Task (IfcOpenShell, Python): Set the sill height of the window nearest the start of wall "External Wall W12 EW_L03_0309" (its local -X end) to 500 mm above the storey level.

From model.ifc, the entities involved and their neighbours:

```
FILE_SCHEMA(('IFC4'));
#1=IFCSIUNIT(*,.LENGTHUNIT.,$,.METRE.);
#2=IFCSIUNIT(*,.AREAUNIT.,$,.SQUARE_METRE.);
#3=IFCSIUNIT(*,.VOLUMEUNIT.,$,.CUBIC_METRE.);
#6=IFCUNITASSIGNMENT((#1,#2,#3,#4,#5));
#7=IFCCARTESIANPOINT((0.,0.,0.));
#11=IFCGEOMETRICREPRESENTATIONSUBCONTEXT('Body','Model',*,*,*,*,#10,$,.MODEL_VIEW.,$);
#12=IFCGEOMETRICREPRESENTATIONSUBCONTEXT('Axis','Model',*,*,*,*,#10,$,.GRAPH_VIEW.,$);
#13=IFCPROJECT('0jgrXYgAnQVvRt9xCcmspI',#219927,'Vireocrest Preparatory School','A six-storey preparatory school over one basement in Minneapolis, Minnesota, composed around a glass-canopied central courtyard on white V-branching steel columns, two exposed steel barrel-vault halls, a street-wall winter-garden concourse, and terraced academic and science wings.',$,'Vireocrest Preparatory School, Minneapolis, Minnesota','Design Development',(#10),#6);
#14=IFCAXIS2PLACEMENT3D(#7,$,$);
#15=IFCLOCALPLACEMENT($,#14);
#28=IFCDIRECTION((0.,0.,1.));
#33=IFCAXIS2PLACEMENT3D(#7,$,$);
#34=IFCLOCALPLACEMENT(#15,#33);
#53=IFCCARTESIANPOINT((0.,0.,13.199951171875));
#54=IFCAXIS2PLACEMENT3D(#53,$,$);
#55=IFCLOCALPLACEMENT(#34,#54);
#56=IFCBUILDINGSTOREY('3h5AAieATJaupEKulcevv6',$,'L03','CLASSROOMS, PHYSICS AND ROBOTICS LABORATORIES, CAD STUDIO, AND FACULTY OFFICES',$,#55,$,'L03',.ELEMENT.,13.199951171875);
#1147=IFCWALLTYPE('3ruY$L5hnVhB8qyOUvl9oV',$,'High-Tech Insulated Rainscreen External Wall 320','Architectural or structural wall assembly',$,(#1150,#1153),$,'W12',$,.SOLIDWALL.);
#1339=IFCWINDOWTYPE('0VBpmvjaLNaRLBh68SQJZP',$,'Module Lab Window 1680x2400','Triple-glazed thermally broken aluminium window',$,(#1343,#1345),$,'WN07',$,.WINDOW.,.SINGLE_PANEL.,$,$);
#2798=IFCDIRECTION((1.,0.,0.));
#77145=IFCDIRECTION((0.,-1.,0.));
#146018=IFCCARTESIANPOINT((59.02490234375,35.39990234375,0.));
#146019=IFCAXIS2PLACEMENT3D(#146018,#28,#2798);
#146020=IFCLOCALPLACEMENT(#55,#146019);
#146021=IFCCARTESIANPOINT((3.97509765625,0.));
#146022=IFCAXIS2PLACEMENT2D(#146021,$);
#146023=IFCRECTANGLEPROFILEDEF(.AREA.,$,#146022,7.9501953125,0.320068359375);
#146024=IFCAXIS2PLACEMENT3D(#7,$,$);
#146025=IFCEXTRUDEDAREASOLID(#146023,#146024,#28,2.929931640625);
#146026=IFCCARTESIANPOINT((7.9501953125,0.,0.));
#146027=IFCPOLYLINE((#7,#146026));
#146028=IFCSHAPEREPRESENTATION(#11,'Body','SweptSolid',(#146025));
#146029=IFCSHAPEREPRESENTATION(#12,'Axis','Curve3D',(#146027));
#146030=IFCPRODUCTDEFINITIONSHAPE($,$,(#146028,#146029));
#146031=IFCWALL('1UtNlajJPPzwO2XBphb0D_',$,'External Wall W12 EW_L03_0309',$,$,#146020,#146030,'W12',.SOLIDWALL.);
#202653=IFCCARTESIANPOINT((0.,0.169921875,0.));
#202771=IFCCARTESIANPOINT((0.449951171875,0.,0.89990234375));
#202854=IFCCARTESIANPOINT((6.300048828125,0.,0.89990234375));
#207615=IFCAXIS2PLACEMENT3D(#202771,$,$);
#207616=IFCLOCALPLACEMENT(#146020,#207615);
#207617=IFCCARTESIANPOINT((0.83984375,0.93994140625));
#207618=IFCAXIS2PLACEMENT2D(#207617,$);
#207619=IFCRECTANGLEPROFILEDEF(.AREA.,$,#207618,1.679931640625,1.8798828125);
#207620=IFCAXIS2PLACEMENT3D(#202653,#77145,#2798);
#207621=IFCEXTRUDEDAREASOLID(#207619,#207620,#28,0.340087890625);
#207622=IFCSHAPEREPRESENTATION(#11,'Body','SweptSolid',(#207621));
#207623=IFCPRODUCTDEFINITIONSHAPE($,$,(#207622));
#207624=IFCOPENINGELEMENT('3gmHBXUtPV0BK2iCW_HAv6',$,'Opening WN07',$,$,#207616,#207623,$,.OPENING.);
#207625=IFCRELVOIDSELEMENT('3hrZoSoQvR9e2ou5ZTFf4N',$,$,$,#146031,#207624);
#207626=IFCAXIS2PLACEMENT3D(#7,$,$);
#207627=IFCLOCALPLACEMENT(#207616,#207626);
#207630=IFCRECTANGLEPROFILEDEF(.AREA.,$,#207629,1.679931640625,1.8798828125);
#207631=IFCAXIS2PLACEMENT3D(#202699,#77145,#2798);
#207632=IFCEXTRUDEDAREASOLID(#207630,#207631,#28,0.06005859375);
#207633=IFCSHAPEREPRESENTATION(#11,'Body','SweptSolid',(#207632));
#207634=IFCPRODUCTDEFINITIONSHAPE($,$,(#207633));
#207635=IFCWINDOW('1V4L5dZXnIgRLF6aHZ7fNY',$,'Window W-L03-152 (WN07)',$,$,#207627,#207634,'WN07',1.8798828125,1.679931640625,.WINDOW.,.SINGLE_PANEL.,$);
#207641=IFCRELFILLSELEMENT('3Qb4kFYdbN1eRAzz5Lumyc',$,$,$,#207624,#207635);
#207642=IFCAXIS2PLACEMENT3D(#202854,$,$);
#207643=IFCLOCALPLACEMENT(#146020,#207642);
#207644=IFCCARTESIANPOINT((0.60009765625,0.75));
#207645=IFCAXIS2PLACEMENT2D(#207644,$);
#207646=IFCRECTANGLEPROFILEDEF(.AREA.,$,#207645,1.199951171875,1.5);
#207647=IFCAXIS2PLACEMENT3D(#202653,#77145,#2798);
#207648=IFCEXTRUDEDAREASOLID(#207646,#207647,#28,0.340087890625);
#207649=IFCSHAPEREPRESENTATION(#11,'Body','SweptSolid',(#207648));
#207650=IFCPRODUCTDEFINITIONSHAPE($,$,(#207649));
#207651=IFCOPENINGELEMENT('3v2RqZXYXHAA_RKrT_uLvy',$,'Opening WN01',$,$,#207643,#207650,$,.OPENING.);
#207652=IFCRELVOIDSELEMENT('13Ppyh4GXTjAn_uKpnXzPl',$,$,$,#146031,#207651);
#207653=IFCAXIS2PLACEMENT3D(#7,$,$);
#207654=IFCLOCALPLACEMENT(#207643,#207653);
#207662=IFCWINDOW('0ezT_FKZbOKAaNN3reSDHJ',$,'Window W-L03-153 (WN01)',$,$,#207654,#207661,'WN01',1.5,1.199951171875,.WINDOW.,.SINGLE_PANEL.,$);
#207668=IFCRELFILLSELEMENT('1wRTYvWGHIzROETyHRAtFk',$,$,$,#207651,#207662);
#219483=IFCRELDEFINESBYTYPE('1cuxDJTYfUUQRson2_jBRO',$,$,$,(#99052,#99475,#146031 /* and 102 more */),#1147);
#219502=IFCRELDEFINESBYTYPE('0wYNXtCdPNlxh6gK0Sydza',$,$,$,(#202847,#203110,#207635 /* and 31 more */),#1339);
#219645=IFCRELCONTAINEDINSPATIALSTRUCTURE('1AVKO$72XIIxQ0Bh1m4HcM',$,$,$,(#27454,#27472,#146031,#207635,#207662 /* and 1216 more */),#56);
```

```python
import numpy as np
import ifcopenshell
import ifcopenshell.api.geometry
import ifcopenshell.geom
import ifcopenshell.util.element
import ifcopenshell.util.placement
import ifcopenshell.util.shape
import ifcopenshell.util.unit

model = ifcopenshell.open("model.ifc")
unit_scale = ifcopenshell.util.unit.calculate_unit_scale(model)

window = model.by_guid("1V4L5dZXnIgRLF6aHZ7fNY")
opening = window.FillsVoids[0].RelatingOpeningElement
storey = ifcopenshell.util.element.get_container(window, ifc_class="IfcBuildingStorey")
level = ifcopenshell.util.placement.get_local_placement(storey.ObjectPlacement)[2, 3]

# The opening's origin need not be at the sill, so measure its lowest point.
shape = ifcopenshell.geom.create_shape(ifcopenshell.geom.settings(), opening)
bottom = ifcopenshell.util.shape.get_shape_bottom_elevation(shape, shape.geometry) / unit_scale
dz = level + 0.5 - bottom

shift = np.array([0.0, 0.0, dz])
# The window is placed relative to its opening, so it follows when the opening moves.
matrix = ifcopenshell.util.placement.get_local_placement(opening.ObjectPlacement)
matrix[:3, 3] += shift
ifcopenshell.api.geometry.edit_object_placement(
    model, product=opening, matrix=matrix, is_si=False, should_transform_children=True
)

print(f"moved by {dz * unit_scale:+.3f} m")

model.write("model_updated.ifc")
```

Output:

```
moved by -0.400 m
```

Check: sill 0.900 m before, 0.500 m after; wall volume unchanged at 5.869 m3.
